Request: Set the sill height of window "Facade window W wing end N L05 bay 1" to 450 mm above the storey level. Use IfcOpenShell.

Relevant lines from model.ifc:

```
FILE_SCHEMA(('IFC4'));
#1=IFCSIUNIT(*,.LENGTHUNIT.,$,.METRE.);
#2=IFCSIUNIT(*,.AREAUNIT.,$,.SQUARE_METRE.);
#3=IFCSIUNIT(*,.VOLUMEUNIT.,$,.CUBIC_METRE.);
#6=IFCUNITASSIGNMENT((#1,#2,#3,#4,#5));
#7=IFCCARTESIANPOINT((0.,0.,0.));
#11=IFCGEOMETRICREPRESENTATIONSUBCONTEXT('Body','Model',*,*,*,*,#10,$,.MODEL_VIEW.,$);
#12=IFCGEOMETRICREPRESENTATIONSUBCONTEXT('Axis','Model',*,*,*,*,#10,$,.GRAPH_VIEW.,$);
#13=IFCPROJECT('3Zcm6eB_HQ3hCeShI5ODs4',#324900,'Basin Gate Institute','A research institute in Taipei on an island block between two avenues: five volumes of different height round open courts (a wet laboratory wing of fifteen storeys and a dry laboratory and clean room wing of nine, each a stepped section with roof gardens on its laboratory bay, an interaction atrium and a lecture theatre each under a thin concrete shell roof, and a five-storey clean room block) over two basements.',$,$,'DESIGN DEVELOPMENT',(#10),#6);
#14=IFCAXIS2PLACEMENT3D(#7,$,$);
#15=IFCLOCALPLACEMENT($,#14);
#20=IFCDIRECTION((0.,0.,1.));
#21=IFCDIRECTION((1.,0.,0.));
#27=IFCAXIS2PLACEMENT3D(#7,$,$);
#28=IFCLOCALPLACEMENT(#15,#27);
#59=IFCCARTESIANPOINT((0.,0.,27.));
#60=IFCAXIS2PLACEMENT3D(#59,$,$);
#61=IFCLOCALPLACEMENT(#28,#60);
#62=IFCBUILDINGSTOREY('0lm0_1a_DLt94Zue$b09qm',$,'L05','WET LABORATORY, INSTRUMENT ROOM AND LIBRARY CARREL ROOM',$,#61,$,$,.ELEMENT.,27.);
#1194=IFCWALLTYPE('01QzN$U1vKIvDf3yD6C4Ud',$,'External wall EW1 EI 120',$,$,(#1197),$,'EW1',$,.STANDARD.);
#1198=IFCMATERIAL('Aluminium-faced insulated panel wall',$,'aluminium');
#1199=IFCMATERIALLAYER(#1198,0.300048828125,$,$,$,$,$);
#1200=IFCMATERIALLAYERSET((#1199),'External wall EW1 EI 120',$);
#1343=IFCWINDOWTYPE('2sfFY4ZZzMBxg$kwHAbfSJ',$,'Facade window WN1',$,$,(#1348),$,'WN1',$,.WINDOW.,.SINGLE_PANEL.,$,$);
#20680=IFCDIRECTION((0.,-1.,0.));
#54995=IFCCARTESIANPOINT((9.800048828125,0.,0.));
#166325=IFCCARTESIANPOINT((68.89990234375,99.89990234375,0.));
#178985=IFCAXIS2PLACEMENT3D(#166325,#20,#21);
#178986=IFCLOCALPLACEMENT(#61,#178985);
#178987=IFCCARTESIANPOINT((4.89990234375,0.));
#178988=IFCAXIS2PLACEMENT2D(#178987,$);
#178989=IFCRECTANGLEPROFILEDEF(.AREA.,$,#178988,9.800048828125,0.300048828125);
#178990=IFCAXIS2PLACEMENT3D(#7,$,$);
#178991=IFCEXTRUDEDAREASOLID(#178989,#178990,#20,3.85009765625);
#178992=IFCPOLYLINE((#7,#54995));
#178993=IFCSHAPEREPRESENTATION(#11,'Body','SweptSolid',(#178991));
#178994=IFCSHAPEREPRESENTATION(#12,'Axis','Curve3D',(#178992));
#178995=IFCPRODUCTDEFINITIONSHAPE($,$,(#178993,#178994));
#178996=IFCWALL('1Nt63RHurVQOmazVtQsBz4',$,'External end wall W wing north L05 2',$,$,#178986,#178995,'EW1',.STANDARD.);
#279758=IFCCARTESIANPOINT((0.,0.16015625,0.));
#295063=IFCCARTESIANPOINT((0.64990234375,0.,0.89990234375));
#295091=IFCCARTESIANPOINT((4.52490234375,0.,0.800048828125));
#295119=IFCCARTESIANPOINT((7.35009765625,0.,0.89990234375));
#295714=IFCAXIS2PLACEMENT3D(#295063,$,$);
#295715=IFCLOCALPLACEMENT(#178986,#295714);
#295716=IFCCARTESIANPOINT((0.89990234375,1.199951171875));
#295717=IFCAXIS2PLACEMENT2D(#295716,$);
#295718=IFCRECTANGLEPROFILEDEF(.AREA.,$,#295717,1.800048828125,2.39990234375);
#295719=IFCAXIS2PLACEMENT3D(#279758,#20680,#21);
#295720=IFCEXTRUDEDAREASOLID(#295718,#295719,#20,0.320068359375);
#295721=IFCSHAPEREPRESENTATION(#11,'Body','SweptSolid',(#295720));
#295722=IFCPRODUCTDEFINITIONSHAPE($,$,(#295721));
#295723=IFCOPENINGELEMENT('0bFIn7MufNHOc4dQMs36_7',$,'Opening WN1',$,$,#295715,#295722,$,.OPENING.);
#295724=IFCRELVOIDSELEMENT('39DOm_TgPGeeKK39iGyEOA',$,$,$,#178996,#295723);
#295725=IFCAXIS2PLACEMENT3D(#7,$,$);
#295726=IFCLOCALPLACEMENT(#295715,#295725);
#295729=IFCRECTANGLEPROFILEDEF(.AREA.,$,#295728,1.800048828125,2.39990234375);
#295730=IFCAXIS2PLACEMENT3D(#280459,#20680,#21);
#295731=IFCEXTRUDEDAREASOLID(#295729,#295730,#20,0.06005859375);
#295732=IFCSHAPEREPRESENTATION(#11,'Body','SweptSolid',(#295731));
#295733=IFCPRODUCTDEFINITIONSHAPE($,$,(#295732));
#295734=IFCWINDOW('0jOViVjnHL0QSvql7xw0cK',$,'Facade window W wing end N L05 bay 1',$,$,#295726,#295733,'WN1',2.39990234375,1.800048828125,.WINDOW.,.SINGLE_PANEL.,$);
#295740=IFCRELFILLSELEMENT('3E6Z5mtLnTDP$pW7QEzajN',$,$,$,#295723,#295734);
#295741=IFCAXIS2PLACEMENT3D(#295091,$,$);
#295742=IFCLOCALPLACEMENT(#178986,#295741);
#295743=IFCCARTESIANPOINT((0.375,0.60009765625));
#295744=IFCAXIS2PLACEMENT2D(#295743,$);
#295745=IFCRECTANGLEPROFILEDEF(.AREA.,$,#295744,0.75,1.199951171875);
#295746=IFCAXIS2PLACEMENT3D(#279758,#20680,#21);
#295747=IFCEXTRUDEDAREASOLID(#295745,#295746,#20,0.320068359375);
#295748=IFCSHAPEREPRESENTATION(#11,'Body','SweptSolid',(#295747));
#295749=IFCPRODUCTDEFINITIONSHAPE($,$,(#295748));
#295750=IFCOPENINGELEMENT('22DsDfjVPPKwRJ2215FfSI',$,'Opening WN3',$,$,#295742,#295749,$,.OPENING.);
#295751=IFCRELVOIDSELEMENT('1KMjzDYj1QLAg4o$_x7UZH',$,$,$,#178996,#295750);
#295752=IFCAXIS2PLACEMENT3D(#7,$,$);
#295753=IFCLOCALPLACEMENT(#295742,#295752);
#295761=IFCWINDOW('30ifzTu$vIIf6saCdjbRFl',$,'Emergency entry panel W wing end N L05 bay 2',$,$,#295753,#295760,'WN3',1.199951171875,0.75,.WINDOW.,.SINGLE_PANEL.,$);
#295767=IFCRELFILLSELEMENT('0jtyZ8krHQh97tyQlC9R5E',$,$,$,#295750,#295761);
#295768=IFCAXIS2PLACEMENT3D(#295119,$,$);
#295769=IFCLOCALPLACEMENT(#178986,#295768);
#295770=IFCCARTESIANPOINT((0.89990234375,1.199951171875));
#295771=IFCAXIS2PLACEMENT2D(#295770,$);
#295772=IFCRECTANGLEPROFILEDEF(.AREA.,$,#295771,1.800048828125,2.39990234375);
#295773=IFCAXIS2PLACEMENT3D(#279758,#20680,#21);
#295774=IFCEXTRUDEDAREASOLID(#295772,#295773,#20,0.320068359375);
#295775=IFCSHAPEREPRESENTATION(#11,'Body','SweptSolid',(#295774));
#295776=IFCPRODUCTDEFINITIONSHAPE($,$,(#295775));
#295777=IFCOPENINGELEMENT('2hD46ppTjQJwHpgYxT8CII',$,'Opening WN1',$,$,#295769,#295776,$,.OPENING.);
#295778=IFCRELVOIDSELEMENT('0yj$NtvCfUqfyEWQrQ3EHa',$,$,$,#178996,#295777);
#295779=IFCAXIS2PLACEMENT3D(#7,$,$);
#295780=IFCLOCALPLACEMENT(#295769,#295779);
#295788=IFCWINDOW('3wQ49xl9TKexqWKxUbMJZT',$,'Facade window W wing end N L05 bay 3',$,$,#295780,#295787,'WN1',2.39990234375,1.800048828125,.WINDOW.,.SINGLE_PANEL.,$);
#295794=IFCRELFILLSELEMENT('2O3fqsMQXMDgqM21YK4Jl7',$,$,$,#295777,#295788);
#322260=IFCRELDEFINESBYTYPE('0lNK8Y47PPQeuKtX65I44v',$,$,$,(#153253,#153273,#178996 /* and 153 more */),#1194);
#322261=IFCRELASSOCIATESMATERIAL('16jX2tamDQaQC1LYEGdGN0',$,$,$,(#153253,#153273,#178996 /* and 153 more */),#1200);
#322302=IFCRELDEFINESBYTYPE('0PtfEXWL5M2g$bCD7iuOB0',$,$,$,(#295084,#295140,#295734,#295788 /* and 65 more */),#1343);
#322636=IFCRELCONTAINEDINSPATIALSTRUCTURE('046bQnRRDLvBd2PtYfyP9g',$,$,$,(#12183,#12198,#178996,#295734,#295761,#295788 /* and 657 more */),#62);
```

```python
import numpy as np
import ifcopenshell
import ifcopenshell.api.geometry
import ifcopenshell.geom
import ifcopenshell.util.element
import ifcopenshell.util.placement
import ifcopenshell.util.shape
import ifcopenshell.util.unit

model = ifcopenshell.open("model.ifc")
unit_scale = ifcopenshell.util.unit.calculate_unit_scale(model)

window = model.by_guid("0jOViVjnHL0QSvql7xw0cK")
opening = window.FillsVoids[0].RelatingOpeningElement
storey = ifcopenshell.util.element.get_container(window, ifc_class="IfcBuildingStorey")
level = ifcopenshell.util.placement.get_local_placement(storey.ObjectPlacement)[2, 3]

# The opening's origin need not be at the sill, so measure its lowest point.
shape = ifcopenshell.geom.create_shape(ifcopenshell.geom.settings(), opening)
bottom = ifcopenshell.util.shape.get_shape_bottom_elevation(shape, shape.geometry) / unit_scale
dz = level + 0.45 / unit_scale - bottom

shift = np.array([0.0, 0.0, dz])
# The window is placed relative to its opening, so it follows when the opening moves.
matrix = ifcopenshell.util.placement.get_local_placement(opening.ObjectPlacement)
matrix[:3, 3] += shift
ifcopenshell.api.geometry.edit_object_placement(
    model, product=opening, matrix=matrix, is_si=False, should_transform_children=True
)

print(f"moved by {dz * unit_scale:+.3f} m")

model.write("model-out.ifc")
```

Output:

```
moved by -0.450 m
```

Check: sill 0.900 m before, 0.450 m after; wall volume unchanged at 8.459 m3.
